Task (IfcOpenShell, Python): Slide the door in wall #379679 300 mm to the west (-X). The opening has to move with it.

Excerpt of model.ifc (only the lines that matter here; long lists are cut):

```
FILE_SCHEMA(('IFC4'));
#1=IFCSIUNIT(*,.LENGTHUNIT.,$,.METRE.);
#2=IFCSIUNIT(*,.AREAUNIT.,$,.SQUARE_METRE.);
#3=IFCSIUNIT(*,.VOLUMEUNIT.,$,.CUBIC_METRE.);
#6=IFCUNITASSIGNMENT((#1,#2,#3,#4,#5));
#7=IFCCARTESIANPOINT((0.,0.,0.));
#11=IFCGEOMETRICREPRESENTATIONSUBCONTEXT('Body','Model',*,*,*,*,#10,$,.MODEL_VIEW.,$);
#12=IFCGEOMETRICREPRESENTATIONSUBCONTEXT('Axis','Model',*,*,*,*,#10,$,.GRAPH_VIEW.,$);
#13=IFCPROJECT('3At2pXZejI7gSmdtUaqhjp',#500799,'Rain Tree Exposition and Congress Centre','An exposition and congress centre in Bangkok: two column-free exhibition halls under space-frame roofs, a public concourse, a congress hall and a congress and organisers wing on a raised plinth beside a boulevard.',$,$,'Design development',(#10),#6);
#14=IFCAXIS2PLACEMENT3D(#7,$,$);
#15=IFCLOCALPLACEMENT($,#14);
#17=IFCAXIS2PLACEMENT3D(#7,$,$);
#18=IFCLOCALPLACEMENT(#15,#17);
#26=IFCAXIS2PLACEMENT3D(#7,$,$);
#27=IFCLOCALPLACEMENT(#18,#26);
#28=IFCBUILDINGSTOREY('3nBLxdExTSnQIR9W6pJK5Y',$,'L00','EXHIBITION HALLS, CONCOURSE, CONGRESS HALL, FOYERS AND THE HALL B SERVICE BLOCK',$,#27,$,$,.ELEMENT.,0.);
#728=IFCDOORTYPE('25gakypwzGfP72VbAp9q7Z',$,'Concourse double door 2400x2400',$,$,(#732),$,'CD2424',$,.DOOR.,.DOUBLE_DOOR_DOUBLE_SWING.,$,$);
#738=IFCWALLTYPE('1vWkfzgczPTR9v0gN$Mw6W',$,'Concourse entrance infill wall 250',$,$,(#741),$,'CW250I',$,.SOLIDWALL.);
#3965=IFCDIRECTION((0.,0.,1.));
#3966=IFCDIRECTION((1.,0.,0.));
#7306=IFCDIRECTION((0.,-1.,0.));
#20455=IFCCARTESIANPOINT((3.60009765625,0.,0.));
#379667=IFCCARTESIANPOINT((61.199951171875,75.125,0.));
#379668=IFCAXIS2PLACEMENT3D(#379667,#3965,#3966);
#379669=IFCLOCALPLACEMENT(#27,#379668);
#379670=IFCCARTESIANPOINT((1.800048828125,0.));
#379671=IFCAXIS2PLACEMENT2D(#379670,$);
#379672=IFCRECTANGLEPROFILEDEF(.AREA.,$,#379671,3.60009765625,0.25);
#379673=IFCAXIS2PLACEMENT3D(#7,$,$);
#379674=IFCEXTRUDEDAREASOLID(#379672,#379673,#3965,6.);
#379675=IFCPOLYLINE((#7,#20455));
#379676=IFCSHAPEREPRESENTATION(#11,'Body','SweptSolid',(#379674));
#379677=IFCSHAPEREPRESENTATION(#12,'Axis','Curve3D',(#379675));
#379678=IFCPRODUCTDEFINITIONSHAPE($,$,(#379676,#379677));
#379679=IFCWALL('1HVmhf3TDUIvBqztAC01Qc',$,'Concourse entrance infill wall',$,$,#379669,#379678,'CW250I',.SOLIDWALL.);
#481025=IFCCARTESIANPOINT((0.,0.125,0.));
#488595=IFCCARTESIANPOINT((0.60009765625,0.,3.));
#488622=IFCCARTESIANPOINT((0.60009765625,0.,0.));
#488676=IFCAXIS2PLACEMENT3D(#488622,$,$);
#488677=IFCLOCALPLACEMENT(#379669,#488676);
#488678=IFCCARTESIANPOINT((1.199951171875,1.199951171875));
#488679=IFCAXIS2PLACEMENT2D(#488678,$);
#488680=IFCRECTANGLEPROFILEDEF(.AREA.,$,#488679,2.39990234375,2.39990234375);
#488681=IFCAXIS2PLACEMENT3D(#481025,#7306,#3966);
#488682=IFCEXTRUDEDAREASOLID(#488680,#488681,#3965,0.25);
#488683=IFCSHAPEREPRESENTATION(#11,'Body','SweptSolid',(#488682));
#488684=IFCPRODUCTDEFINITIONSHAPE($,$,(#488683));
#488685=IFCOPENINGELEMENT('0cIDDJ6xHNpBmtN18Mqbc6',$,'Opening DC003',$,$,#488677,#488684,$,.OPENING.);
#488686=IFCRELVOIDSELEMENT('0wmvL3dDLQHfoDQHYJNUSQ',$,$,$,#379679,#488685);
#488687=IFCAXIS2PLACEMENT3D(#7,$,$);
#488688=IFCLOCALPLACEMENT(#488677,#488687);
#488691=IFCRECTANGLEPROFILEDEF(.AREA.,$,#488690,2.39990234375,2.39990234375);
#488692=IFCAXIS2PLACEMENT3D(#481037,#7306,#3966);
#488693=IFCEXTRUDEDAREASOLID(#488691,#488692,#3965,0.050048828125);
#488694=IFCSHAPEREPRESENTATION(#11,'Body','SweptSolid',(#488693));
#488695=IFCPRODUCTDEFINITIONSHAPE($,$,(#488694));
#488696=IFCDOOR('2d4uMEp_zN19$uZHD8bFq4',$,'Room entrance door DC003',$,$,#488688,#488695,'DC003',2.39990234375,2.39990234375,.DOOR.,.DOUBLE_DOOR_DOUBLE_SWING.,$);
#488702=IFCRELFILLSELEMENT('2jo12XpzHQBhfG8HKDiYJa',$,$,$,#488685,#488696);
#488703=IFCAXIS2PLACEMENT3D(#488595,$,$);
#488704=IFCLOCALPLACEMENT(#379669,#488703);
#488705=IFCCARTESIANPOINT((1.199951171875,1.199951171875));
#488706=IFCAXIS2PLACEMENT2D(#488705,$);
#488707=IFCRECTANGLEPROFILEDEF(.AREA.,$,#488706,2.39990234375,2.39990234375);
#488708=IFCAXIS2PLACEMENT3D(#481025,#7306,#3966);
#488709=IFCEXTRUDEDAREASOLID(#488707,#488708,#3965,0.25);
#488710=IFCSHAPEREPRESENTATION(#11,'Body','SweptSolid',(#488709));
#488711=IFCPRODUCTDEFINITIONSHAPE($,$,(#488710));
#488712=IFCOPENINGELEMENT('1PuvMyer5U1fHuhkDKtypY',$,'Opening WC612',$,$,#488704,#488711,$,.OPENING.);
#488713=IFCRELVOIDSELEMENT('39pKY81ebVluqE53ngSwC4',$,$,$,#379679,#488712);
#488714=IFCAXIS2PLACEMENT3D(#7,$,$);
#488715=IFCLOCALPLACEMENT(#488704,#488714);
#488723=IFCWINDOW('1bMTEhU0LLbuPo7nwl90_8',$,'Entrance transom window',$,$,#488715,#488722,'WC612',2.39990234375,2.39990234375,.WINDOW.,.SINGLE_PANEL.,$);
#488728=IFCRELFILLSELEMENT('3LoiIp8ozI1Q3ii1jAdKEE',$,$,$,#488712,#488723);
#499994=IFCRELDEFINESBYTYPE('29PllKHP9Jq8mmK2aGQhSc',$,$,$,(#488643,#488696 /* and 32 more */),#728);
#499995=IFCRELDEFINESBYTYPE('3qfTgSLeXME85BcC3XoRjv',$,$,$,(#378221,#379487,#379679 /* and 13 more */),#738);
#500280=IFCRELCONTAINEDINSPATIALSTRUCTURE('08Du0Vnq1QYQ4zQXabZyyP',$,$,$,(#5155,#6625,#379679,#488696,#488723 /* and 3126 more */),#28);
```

```python
import ifcopenshell
import ifcopenshell.api.geometry
import ifcopenshell.util.placement
import ifcopenshell.util.unit

model = ifcopenshell.open("model.ifc")
unit_scale = ifcopenshell.util.unit.calculate_unit_scale(model)

door = model.by_id(488696)
opening = door.FillsVoids[0].RelatingOpeningElement
wall = opening.VoidsElements[0].RelatingBuildingElement

wall_matrix = ifcopenshell.util.placement.get_local_placement(wall.ObjectPlacement)
shift = wall_matrix[:3, 0] * -0.3 / unit_scale
before = ifcopenshell.util.placement.get_local_placement(door.ObjectPlacement)[:3, 3].copy()

# The door is placed relative to its opening, so it follows when the opening moves.
matrix = ifcopenshell.util.placement.get_local_placement(opening.ObjectPlacement)
matrix[:3, 3] += shift
ifcopenshell.api.geometry.edit_object_placement(
    model, product=opening, matrix=matrix, is_si=False, should_transform_children=True
)

after = ifcopenshell.util.placement.get_local_placement(door.ObjectPlacement)[:3, 3]
print("door moved by", (after - before).round(3) + 0.0)

model.write("model_edited.ifc")
```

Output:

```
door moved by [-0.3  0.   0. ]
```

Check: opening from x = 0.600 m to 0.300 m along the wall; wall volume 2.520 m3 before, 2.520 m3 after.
